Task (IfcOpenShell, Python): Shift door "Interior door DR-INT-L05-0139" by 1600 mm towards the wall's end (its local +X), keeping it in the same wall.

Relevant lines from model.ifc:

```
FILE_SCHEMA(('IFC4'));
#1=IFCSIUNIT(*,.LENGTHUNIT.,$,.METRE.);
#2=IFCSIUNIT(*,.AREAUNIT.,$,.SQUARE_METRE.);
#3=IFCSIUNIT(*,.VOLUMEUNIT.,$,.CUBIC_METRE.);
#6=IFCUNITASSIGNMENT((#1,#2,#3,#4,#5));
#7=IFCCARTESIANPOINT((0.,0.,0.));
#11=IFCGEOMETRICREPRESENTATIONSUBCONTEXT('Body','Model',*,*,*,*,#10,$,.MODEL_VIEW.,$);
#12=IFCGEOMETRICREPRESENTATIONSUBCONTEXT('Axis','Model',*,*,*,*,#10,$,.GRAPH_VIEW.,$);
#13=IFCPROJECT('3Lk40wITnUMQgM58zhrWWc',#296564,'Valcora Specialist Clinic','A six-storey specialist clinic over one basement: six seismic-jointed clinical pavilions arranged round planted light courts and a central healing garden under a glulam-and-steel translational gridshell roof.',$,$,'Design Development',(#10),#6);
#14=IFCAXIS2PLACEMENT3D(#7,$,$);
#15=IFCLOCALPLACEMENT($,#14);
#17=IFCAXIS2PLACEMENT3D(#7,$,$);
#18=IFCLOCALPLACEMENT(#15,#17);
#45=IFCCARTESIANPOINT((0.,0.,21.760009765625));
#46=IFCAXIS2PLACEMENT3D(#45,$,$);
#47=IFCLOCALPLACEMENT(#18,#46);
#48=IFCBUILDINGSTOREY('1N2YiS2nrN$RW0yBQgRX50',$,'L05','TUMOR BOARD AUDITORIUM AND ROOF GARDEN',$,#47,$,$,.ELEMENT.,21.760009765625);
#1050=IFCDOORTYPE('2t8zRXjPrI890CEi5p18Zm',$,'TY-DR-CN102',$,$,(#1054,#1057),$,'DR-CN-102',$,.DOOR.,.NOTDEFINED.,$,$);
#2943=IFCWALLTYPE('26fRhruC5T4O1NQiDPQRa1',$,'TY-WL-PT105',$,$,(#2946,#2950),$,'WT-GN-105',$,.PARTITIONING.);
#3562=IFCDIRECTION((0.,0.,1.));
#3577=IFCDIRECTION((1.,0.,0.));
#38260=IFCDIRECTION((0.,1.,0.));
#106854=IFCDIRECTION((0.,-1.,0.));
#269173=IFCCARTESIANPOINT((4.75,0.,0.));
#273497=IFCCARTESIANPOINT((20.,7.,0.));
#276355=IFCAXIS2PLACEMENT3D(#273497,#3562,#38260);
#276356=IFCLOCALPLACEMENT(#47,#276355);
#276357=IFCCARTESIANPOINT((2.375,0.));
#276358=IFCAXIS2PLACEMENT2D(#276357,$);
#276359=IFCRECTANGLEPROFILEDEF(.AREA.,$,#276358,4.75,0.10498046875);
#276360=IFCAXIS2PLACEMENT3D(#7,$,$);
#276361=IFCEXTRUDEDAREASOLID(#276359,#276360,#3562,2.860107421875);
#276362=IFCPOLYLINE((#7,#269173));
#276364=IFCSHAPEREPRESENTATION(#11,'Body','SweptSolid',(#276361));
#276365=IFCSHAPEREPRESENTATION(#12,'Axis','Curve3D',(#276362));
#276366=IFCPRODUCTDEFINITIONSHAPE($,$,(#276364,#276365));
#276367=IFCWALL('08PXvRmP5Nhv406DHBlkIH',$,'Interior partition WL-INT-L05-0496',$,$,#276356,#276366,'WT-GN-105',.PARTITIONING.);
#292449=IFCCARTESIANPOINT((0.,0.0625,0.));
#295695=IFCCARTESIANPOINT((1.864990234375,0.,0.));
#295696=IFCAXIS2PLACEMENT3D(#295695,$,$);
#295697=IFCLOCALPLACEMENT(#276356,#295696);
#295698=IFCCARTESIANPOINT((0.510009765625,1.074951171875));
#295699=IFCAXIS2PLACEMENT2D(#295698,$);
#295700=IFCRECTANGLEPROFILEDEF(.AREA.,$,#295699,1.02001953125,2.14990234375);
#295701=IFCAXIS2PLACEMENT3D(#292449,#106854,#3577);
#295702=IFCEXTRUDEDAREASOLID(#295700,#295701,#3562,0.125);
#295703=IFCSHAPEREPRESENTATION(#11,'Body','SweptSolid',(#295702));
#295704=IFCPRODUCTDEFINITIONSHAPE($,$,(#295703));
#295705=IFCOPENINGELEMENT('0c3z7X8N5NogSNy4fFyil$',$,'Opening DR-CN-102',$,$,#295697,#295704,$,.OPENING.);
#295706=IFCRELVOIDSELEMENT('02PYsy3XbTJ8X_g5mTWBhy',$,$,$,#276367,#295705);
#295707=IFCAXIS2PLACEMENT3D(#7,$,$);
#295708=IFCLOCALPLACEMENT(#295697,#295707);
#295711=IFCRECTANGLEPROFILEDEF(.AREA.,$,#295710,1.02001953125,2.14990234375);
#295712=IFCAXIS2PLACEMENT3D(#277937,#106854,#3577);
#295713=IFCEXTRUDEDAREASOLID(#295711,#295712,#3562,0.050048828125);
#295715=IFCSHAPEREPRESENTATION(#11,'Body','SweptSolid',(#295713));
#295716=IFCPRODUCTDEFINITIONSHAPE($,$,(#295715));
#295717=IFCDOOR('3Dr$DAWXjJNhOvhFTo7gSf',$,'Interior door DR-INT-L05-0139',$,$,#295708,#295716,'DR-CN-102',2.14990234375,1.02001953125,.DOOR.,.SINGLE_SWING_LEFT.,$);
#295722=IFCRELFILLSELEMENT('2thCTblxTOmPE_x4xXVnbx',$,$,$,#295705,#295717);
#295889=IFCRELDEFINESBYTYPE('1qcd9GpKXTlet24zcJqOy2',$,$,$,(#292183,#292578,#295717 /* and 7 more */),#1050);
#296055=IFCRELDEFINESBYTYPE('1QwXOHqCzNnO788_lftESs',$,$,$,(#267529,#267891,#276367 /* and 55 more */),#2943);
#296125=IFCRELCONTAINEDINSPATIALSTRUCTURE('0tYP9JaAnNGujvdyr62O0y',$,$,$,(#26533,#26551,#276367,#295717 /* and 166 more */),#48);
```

```python
import ifcopenshell
import ifcopenshell.api.geometry
import ifcopenshell.util.placement
import ifcopenshell.util.unit

model = ifcopenshell.open("model.ifc")
unit_scale = ifcopenshell.util.unit.calculate_unit_scale(model)

door = model.by_guid("3Dr$DAWXjJNhOvhFTo7gSf")
opening = door.FillsVoids[0].RelatingOpeningElement
wall = opening.VoidsElements[0].RelatingBuildingElement

wall_matrix = ifcopenshell.util.placement.get_local_placement(wall.ObjectPlacement)
shift = wall_matrix[:3, 0] * 1.6 / unit_scale
before = ifcopenshell.util.placement.get_local_placement(door.ObjectPlacement)[:3, 3].copy()

# The door is placed relative to its opening, so it follows when the opening moves.
matrix = ifcopenshell.util.placement.get_local_placement(opening.ObjectPlacement)
matrix[:3, 3] += shift
ifcopenshell.api.geometry.edit_object_placement(
    model, product=opening, matrix=matrix, is_si=False, should_transform_children=True
)

after = ifcopenshell.util.placement.get_local_placement(door.ObjectPlacement)[:3, 3]
print("door moved by", (after - before).round(3) + 0.0)

model.write("model_edited.ifc")
```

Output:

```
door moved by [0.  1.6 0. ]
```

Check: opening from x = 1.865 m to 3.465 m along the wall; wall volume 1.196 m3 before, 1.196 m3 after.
